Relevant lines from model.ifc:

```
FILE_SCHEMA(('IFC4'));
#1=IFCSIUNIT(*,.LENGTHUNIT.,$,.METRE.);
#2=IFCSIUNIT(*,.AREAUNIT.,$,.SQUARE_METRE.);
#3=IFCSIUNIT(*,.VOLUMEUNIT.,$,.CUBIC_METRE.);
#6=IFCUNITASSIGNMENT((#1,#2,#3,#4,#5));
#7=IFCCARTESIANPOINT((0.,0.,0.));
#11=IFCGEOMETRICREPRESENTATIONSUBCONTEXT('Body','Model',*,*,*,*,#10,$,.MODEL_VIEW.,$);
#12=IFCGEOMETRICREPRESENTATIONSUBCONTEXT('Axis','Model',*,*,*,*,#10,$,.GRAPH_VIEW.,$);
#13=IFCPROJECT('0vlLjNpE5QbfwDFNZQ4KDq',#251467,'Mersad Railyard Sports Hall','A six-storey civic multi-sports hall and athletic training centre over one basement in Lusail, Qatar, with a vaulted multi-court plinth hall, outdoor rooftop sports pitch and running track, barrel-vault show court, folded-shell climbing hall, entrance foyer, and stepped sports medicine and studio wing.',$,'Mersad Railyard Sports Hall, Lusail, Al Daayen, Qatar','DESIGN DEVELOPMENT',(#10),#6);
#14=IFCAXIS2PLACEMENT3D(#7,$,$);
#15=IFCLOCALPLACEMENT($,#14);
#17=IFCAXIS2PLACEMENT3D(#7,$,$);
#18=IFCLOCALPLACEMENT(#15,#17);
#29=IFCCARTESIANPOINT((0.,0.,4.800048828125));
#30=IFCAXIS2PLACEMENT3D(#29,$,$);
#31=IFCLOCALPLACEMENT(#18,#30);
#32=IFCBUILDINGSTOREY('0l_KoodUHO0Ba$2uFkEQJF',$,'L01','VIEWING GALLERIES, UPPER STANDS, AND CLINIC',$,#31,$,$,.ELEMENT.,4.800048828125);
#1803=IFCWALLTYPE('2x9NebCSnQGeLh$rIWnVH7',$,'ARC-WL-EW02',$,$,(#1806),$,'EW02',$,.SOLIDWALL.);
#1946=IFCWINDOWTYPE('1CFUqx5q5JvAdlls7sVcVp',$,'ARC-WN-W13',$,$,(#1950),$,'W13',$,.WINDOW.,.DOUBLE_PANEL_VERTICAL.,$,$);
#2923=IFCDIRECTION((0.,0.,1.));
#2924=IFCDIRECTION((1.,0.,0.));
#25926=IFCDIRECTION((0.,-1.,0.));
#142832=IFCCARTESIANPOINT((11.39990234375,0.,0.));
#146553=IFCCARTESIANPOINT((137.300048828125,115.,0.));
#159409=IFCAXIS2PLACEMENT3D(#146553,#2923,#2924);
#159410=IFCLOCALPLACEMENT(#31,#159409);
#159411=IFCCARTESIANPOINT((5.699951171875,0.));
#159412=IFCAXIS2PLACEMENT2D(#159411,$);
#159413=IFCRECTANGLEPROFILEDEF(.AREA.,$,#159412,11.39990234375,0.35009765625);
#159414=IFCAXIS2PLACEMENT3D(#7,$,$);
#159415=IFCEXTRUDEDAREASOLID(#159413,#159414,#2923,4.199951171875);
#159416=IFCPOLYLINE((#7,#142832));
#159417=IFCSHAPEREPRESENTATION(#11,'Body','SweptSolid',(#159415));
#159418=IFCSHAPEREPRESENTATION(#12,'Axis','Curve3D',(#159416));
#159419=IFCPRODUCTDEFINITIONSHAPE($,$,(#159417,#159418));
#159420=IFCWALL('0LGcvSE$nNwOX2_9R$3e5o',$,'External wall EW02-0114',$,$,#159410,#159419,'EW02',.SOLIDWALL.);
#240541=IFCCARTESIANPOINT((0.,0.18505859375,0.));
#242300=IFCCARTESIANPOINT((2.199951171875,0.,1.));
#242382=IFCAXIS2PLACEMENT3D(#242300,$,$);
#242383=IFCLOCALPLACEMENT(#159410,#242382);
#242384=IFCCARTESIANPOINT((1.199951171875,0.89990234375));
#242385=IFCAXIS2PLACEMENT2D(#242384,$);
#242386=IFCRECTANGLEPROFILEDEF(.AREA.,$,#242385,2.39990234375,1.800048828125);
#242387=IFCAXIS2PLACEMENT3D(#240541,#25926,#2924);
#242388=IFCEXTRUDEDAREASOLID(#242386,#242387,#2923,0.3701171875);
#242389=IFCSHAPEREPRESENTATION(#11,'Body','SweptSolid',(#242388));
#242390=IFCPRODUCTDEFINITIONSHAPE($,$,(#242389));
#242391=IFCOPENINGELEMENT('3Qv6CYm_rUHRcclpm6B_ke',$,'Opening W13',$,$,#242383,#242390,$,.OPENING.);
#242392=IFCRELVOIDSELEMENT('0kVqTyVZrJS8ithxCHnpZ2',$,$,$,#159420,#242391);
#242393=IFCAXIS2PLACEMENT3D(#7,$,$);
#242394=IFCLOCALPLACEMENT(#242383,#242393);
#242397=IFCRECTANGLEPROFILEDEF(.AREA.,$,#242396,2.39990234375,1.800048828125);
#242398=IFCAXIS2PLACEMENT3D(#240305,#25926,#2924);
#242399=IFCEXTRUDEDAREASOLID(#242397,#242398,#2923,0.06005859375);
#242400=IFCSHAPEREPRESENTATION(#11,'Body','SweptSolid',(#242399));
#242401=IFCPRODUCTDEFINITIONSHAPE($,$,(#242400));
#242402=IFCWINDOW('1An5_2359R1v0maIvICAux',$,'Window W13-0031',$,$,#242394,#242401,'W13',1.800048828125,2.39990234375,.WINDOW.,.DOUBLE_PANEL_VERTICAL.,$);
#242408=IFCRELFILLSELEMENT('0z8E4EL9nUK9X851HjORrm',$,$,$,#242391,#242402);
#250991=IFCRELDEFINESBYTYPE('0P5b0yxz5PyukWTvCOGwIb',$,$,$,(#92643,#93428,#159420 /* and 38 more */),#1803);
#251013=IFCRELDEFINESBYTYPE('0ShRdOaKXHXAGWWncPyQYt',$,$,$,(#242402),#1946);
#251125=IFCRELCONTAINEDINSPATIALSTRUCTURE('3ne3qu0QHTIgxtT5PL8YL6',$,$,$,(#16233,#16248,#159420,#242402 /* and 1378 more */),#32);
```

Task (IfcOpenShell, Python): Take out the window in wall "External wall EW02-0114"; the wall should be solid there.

```python
import ifcopenshell
import ifcopenshell.api.feature
import ifcopenshell.api.root
import ifcopenshell.geom
import ifcopenshell.util.shape

model = ifcopenshell.open("model.ifc")
settings = ifcopenshell.geom.settings()


def volume(element):
    """Net volume in cubic metres, openings subtracted."""
    shape = ifcopenshell.geom.create_shape(settings, element)
    return ifcopenshell.util.shape.get_volume(shape.geometry)


window = model.by_guid("1An5_2359R1v0maIvICAux")
opening = window.FillsVoids[0].RelatingOpeningElement
wall = opening.VoidsElements[0].RelatingBuildingElement
before = volume(wall)

ifcopenshell.api.root.remove_product(model, product=window)
ifcopenshell.api.feature.remove_feature(model, feature=opening)

after = volume(wall)

print(f"wall volume {before:.3f} -> {after:.3f} m3")

model.write("model_rev.ifc")
```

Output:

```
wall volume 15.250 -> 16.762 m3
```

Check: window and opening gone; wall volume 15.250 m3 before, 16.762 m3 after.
